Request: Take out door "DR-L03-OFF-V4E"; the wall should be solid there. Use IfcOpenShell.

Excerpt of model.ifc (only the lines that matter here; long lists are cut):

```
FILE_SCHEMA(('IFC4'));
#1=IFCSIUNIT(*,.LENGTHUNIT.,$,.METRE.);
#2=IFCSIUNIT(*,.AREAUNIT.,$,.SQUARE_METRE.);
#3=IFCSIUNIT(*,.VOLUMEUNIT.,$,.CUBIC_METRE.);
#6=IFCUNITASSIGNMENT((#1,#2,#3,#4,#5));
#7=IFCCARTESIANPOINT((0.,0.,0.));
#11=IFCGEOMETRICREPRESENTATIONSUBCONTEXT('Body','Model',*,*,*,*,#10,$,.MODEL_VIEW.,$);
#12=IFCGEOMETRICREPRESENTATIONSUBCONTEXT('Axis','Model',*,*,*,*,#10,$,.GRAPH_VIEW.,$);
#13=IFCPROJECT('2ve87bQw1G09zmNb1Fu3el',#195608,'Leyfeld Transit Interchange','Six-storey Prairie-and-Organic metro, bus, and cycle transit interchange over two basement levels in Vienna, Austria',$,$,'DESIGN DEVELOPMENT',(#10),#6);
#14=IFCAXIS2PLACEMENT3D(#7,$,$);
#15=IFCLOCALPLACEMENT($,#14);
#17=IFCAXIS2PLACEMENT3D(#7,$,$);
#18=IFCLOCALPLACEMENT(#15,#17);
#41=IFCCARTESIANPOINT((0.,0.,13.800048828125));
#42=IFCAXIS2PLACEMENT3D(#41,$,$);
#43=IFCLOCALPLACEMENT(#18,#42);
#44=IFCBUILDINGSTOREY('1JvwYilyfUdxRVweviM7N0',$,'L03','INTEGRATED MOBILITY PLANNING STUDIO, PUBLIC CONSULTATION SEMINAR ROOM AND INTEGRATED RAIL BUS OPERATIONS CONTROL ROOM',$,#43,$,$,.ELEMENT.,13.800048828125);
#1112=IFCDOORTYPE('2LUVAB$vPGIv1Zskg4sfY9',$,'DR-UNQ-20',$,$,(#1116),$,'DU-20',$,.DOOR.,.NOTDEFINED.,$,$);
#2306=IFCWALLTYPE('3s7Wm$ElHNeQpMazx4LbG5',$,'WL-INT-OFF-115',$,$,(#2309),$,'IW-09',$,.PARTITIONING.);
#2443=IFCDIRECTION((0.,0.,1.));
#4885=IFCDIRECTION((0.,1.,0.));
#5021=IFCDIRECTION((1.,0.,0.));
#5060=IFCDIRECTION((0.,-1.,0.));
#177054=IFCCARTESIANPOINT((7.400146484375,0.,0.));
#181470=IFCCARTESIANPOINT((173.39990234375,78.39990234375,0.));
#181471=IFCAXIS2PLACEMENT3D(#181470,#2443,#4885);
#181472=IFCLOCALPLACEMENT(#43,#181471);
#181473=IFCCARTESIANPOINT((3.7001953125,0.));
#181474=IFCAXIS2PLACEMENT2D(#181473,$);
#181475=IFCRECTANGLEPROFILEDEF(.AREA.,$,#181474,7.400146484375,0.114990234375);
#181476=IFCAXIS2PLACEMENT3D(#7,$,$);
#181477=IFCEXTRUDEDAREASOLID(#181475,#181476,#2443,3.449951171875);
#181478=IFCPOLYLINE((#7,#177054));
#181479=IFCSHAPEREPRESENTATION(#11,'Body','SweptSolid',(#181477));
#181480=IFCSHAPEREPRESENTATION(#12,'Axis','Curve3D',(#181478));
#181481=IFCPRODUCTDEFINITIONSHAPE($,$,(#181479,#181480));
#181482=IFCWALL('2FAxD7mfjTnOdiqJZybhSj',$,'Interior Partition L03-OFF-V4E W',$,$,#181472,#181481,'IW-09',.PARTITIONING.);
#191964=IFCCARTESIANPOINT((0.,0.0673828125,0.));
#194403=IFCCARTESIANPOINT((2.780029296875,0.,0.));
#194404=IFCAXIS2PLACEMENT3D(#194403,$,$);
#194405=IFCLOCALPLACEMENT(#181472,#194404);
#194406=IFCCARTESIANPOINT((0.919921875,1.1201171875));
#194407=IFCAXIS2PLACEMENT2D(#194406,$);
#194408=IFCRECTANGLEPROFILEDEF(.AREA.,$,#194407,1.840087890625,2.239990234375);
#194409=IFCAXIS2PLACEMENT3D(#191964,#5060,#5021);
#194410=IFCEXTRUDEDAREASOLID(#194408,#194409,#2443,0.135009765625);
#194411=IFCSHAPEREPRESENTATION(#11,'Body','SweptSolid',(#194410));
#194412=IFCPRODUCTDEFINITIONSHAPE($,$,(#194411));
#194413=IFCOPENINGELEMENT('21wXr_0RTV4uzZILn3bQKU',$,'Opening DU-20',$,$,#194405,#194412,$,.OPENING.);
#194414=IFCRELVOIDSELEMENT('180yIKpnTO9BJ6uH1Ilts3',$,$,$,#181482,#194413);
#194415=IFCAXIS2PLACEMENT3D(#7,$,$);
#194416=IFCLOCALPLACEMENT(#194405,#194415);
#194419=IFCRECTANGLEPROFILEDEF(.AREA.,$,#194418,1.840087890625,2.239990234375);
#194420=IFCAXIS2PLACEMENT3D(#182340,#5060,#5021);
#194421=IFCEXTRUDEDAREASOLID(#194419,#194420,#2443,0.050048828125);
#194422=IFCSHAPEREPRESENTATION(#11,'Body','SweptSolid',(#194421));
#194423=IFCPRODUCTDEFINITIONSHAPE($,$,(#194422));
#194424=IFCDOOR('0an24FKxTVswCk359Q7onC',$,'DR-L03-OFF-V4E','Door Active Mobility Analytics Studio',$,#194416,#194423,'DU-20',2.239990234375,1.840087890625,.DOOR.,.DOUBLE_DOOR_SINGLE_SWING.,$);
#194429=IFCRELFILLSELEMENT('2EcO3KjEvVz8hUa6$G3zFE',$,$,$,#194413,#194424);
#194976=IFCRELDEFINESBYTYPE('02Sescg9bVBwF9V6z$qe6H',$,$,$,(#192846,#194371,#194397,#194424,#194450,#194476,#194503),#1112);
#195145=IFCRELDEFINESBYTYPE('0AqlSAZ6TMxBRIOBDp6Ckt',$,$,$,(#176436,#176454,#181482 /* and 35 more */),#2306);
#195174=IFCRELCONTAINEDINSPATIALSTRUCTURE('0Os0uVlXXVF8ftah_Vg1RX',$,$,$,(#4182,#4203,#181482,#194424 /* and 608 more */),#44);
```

```python
import ifcopenshell
import ifcopenshell.api.feature
import ifcopenshell.api.root
import ifcopenshell.geom
import ifcopenshell.util.shape

model = ifcopenshell.open("model.ifc")
settings = ifcopenshell.geom.settings()


def volume(element):
    """Net volume in cubic metres, openings subtracted."""
    shape = ifcopenshell.geom.create_shape(settings, element)
    return ifcopenshell.util.shape.get_volume(shape.geometry)


door = model.by_guid("0an24FKxTVswCk359Q7onC")
opening = door.FillsVoids[0].RelatingOpeningElement
wall = opening.VoidsElements[0].RelatingBuildingElement
before = volume(wall)

ifcopenshell.api.root.remove_product(model, product=door)
ifcopenshell.api.feature.remove_feature(model, feature=opening)

after = volume(wall)

print(f"wall volume {before:.3f} -> {after:.3f} m3")

model.write("model_rev.ifc")
```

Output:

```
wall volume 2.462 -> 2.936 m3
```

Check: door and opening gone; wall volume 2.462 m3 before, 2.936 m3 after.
